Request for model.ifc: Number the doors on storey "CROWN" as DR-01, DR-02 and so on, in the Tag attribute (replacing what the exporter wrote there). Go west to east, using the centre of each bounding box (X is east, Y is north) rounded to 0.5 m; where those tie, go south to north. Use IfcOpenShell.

First a look at what the model holds.

```python
import ifcopenshell
import ifcopenshell.util.element
import ifcopenshell.util.placement

model = ifcopenshell.open("model.ifc")
print(model.schema)
storey = next(s for s in model.by_type("IfcBuildingStorey") if s.Name == "CROWN")
doors = [e for e in ifcopenshell.util.element.get_decomposition(storey) if e.is_a("IfcDoor")]
for e in sorted(doors, key=lambda e: e.id()):
    origin = ifcopenshell.util.placement.get_local_placement(e.ObjectPlacement)[:3, 3]
    print(e.id(), e.Tag, e.Name, origin.round(2) + 0.0, sep=" | ")
```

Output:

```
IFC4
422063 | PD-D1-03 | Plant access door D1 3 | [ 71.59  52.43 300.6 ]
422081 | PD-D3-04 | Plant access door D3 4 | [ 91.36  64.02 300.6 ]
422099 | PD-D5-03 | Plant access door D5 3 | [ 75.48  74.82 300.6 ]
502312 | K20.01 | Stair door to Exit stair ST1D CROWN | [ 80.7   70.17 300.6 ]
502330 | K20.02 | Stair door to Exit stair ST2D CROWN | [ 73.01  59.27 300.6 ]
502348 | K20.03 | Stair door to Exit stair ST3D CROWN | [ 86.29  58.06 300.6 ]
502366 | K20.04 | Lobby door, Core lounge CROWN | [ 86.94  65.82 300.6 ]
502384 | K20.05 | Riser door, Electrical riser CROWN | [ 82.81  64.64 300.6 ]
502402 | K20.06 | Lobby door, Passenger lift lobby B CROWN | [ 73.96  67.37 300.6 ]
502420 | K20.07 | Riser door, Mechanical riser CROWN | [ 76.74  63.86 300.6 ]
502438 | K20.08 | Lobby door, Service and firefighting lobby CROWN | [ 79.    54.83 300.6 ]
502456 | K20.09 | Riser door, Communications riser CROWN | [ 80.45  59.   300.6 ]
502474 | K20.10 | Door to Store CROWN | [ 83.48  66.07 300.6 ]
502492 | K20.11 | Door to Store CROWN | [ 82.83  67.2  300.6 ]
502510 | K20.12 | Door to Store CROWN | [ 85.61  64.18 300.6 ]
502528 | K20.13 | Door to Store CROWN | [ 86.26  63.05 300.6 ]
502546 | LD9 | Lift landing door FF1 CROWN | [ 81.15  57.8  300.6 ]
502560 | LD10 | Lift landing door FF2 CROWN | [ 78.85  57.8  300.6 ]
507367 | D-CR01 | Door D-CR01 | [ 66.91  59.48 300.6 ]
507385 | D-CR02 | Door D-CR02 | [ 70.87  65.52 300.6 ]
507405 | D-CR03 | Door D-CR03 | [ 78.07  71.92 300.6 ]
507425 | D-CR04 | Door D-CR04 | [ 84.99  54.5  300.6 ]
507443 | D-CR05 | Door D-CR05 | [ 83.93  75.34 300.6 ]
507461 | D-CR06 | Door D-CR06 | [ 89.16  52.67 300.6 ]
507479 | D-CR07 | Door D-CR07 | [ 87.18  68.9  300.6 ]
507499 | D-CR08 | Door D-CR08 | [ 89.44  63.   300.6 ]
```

```python
import ifcopenshell
import ifcopenshell.geom
import ifcopenshell.util.element
import ifcopenshell.util.shape

model = ifcopenshell.open("model.ifc")
settings = ifcopenshell.geom.settings()
settings.set("use-world-coords", True)


def centre(element):
    shape = ifcopenshell.geom.create_shape(settings, element)
    return ifcopenshell.util.shape.get_bbox_centroid(shape.geometry)


storey = next(s for s in model.by_type("IfcBuildingStorey") if s.Name == "CROWN")
doors = [e for e in ifcopenshell.util.element.get_decomposition(storey) if e.is_a("IfcDoor")]

# Insertion points can sit at a corner or the storey origin, so sort by the geometry (in metres).
centres = {e: centre(e) for e in doors}
doors.sort(key=lambda e: (round(centres[e][0] / 0.5), centres[e][1]))

for i, e in enumerate(doors, start=1):
    number = f"DR-{i:02d}"
    e.Tag = number
    print(e.id(), number)

model.write("model_v2.ifc")
```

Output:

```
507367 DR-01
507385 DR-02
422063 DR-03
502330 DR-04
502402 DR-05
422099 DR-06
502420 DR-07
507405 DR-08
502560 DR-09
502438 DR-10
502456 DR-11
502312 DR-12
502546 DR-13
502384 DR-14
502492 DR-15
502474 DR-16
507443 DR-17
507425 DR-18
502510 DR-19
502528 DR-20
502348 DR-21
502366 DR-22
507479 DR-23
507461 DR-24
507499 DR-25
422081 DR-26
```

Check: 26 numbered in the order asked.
